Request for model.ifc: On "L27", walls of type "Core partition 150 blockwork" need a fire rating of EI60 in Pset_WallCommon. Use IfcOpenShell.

First a look at what the model holds.

```python
import ifcopenshell
import ifcopenshell.util.element

model = ifcopenshell.open("model.ifc")
print(model.schema)
storey = next(s for s in model.by_type("IfcBuildingStorey") if s.Name == "L27")
walls = [e for e in ifcopenshell.util.element.get_decomposition(storey) if e.is_a("IfcWall")]
seen = {}
for e in walls:
    element_type = ifcopenshell.util.element.get_type(e)
    key = (element_type.Name if element_type != e and element_type else None, ifcopenshell.util.element.get_pset(e, "Pset_WallCommon", "FireRating"))
    seen[key] = seen.get(key, 0) + 1
for (name, value), count in sorted(seen.items(), key=str):
    print(count, "x", name, "|", value)
```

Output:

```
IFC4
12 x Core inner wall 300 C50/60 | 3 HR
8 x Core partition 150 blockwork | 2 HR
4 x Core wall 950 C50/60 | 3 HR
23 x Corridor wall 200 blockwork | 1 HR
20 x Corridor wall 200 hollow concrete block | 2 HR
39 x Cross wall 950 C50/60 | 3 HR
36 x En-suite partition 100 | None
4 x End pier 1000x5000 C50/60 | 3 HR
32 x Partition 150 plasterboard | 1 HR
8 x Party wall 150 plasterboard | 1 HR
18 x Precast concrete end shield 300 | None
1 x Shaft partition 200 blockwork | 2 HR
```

```python
import ifcopenshell
import ifcopenshell.api.pset
import ifcopenshell.util.element

model = ifcopenshell.open("model.ifc")

storey = next(s for s in model.by_type("IfcBuildingStorey") if s.Name == "L27")
walls = [e for e in ifcopenshell.util.element.get_decomposition(storey) if e.is_a("IfcWall")]

count = 0
for e in walls:
    element_type = ifcopenshell.util.element.get_type(e)
    if element_type in (None, e) or element_type.Name != "Core partition 150 blockwork":
        continue
    found = ifcopenshell.util.element.get_pset(e, "Pset_WallCommon", should_inherit=False)
    if found:
        pset = model.by_id(found["id"])
        if len(ifcopenshell.util.element.get_elements_by_pset(pset)) > 1:
            pset = ifcopenshell.api.pset.unshare_pset(model, products=[e], pset=pset)[0]
    else:
        pset = ifcopenshell.api.pset.add_pset(model, product=e, name="Pset_WallCommon")
    ifcopenshell.api.pset.edit_pset(model, pset=pset, properties={"FireRating": "EI60"})
    count += 1

print(count, "walls updated")

model.write("model-out.ifc")
```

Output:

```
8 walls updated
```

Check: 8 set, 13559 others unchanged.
